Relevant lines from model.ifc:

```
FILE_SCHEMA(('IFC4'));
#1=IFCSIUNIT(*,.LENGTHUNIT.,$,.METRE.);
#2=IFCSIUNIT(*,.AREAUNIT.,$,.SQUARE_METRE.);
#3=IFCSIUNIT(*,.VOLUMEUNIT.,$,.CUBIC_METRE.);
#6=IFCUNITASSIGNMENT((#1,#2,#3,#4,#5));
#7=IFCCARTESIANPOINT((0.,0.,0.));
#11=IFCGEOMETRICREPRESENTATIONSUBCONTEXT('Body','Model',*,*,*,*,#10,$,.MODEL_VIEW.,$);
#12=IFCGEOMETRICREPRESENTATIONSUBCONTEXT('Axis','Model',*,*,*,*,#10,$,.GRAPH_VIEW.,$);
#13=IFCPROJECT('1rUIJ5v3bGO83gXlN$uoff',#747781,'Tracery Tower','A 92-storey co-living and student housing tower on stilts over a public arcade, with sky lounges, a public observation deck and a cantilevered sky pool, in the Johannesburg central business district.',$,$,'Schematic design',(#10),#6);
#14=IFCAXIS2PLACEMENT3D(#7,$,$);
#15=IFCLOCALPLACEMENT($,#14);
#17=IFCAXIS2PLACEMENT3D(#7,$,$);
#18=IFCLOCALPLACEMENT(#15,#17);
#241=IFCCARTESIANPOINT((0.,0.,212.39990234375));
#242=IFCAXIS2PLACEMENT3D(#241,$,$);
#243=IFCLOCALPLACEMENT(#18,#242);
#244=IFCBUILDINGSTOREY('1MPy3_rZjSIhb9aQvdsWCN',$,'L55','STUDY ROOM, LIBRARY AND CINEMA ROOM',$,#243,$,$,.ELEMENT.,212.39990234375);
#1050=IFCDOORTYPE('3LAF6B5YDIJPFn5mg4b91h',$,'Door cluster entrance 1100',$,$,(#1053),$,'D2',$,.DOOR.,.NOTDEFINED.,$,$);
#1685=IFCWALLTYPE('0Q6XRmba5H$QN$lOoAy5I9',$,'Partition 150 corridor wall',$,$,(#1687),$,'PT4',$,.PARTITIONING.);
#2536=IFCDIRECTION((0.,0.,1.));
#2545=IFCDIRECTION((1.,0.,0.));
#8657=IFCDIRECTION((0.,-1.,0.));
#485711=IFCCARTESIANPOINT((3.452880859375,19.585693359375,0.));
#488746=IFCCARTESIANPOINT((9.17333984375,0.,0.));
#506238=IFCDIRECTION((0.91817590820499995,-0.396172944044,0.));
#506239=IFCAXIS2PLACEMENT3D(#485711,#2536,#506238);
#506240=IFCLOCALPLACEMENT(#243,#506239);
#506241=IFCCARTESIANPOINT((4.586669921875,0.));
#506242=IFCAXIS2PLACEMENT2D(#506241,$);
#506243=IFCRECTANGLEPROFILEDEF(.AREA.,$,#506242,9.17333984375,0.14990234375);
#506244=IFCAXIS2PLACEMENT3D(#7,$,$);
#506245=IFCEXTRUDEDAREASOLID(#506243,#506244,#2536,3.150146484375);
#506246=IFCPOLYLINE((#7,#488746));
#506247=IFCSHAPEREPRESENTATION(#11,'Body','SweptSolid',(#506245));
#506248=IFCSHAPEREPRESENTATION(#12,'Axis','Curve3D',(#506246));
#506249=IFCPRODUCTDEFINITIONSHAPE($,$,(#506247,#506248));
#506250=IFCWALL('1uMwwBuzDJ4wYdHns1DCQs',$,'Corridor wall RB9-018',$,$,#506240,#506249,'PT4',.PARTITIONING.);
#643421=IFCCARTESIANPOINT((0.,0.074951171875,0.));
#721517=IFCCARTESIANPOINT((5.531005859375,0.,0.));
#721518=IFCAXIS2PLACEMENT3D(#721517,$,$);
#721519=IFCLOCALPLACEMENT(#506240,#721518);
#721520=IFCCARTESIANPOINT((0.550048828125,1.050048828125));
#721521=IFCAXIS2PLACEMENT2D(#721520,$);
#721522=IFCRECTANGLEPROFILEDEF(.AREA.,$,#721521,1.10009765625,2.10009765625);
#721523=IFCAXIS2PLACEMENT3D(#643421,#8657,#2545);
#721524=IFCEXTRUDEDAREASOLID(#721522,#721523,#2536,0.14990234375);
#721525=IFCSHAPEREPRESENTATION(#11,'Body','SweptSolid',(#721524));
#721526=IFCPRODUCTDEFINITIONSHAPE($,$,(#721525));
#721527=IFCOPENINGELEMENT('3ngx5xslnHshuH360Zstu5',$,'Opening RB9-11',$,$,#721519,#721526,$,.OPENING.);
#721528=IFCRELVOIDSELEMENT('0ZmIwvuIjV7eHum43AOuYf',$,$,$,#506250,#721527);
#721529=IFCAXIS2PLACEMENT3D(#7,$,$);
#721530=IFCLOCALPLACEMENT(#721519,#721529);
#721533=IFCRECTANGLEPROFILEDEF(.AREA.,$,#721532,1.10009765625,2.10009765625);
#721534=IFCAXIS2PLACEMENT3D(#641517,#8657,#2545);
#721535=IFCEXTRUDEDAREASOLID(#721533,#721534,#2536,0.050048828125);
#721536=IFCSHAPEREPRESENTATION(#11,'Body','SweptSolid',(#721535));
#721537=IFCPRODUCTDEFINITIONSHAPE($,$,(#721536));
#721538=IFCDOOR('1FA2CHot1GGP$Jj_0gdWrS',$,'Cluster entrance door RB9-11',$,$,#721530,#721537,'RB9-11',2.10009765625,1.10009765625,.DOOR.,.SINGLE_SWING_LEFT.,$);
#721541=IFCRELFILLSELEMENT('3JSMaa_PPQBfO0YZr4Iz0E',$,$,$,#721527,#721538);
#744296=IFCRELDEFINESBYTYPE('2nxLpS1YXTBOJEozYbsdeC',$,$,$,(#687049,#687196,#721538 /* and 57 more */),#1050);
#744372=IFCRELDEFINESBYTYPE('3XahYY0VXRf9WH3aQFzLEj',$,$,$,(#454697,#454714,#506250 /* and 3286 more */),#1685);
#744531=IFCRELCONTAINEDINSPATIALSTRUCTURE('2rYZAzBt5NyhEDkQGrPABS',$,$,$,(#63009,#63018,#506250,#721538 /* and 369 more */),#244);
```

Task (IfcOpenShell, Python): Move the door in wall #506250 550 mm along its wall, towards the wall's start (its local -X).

```python
import ifcopenshell
import ifcopenshell.api.geometry
import ifcopenshell.util.placement

model = ifcopenshell.open("model.ifc")

door = model.by_id(721538)
opening = door.FillsVoids[0].RelatingOpeningElement
wall = opening.VoidsElements[0].RelatingBuildingElement

wall_matrix = ifcopenshell.util.placement.get_local_placement(wall.ObjectPlacement)
shift = wall_matrix[:3, 0] * -0.55
before = ifcopenshell.util.placement.get_local_placement(door.ObjectPlacement)[:3, 3].copy()

# The door is placed relative to its opening, so it follows when the opening moves.
matrix = ifcopenshell.util.placement.get_local_placement(opening.ObjectPlacement)
matrix[:3, 3] += shift
ifcopenshell.api.geometry.edit_object_placement(
    model, product=opening, matrix=matrix, is_si=False, should_transform_children=True
)

after = ifcopenshell.util.placement.get_local_placement(door.ObjectPlacement)[:3, 3]
print("door moved by", (after - before).round(3) + 0.0)

model.write("model_edited.ifc")
```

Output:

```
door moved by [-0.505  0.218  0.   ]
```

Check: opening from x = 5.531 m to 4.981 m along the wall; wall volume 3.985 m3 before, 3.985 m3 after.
